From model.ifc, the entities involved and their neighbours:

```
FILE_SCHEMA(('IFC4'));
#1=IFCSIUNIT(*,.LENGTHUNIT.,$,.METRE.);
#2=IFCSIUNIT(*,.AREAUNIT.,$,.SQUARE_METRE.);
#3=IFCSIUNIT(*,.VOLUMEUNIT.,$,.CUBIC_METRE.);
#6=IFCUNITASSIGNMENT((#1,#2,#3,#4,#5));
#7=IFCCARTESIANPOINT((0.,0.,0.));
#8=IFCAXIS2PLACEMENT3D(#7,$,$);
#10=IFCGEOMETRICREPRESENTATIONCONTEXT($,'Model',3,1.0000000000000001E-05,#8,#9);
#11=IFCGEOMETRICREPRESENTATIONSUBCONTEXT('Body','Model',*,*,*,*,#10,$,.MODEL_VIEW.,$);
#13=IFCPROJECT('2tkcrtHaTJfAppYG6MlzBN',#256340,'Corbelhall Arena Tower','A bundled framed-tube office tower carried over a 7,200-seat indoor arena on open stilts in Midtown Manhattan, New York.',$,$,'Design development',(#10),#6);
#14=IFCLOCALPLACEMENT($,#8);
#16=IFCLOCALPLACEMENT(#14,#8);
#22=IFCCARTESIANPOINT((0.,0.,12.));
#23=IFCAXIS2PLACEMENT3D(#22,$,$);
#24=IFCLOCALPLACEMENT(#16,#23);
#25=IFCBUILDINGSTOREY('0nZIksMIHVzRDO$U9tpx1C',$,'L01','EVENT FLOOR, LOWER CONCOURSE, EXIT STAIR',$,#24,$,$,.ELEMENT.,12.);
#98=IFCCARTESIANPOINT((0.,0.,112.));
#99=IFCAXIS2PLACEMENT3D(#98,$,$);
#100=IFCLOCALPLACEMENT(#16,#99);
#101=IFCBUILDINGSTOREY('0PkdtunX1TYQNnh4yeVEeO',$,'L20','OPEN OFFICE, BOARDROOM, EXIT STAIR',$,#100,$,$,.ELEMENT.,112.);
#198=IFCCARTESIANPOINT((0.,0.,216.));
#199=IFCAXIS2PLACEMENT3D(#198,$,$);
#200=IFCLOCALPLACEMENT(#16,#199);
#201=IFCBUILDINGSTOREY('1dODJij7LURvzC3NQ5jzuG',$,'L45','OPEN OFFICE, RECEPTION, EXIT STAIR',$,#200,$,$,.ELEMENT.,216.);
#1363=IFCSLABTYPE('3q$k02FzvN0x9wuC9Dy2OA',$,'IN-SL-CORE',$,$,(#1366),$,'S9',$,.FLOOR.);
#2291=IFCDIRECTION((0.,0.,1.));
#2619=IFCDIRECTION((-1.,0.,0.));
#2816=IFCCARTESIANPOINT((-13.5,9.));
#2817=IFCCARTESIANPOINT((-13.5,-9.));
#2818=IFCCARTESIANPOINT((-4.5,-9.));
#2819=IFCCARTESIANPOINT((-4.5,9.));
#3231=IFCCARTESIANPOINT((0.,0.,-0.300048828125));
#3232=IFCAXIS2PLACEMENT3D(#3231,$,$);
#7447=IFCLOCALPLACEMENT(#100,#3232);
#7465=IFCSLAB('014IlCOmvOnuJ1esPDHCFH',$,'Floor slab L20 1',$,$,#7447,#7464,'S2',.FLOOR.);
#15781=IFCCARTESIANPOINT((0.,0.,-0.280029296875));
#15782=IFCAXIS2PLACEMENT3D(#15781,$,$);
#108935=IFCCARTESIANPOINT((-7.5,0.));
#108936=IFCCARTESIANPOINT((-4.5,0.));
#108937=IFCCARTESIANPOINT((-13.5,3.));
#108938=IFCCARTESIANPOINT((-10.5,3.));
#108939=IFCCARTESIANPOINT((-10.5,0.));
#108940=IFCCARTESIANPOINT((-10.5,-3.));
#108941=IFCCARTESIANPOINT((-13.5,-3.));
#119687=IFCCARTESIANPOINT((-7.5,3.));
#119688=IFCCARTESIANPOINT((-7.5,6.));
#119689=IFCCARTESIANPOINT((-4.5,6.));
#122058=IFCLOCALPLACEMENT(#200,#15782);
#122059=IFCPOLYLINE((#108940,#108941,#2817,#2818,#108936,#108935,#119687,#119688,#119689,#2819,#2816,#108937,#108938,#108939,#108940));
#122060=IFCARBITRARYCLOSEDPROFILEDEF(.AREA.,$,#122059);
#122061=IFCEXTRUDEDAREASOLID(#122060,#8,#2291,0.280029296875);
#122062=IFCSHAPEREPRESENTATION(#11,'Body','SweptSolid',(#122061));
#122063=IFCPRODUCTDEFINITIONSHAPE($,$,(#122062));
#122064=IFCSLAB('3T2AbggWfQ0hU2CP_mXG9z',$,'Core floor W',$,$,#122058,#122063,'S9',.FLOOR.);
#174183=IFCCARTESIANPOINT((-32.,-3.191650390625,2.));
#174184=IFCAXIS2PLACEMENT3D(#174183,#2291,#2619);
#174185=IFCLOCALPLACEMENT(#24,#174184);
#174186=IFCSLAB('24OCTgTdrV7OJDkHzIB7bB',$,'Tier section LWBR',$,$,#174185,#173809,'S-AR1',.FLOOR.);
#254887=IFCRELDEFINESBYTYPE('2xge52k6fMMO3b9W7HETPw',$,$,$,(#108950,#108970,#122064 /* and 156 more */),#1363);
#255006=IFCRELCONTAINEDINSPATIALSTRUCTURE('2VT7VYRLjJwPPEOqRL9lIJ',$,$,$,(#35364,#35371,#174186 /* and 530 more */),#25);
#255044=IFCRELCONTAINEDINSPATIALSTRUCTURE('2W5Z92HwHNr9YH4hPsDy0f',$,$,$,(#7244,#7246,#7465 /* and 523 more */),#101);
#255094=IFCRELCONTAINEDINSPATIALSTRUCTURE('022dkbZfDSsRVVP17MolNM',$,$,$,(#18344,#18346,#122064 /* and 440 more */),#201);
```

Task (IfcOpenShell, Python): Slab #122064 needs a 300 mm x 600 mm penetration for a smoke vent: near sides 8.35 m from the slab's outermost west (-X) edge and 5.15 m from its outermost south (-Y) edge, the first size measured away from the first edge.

```python
import numpy as np
import ifcopenshell
import ifcopenshell.api.feature
import ifcopenshell.api.geometry
import ifcopenshell.api.root
import ifcopenshell.geom
import ifcopenshell.util.placement
import ifcopenshell.util.representation
import ifcopenshell.util.shape
import ifcopenshell.util.unit

model = ifcopenshell.open("model.ifc")
unit_scale = ifcopenshell.util.unit.calculate_unit_scale(model)
settings = ifcopenshell.geom.settings()


def volume(element):
    """Net volume in cubic metres, openings subtracted."""
    shape = ifcopenshell.geom.create_shape(settings, element)
    return ifcopenshell.util.shape.get_volume(shape.geometry)


slab = model.by_guid("3T2AbggWfQ0hU2CP_mXG9z")
before = volume(slab)

# Extent in the slab's own axes, in metres. The edges named are its -X and -Y sides.
slab_shape = ifcopenshell.geom.create_shape(settings, slab)
vertices = ifcopenshell.util.shape.get_vertices(slab_shape.geometry)
x_min, y_min, bottom = vertices.min(axis=0)
top = vertices[:, 2].max()

opening = ifcopenshell.api.root.create_entity(model, ifc_class="IfcOpeningElement", name="Smoke vent opening", predefined_type="OPENING")
context = ifcopenshell.util.representation.get_context(model, "Model", "Body", "MODEL_VIEW")
width, depth = 0.3, 0.6
outline = [(0.0, 0.0), (width, 0.0), (width, depth), (0.0, depth), (0.0, 0.0)]
# Overshoot both faces by 50 mm so the cut is clean.
shape = ifcopenshell.api.geometry.add_slab_representation(
    model, context=context, depth=top - bottom + 0.1, polyline=outline
)
ifcopenshell.api.geometry.assign_representation(model, product=opening, representation=shape)

matrix = ifcopenshell.util.placement.get_local_placement(slab.ObjectPlacement)
matrix[:, 3] = matrix @ np.append(np.array([x_min + 8.35, y_min + 5.15, bottom - 0.05]) / unit_scale, 1.0)
ifcopenshell.api.geometry.edit_object_placement(model, product=opening, matrix=matrix, is_si=False)
ifcopenshell.api.feature.add_feature(model, feature=opening, element=slab)

after = volume(slab)

print(f"slab volume {before:.3f} -> {after:.3f} m3")

model.write("model_rev.ifc")
```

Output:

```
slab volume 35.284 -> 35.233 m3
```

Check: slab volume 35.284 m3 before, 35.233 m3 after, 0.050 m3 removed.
